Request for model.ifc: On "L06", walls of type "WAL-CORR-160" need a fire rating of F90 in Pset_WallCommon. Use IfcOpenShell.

First a look at what the model holds.

```python
import ifcopenshell
import ifcopenshell.util.element

model = ifcopenshell.open("model.ifc")
print(model.schema)
storey = next(s for s in model.by_type("IfcBuildingStorey") if s.Name == "L06")
walls = [e for e in ifcopenshell.util.element.get_decomposition(storey) if e.is_a("IfcWall")]
seen = {}
for e in walls:
    element_type = ifcopenshell.util.element.get_type(e)
    key = (element_type.Name if element_type != e and element_type else None, ifcopenshell.util.element.get_pset(e, "Pset_WallCommon", "FireRating"))
    seen[key] = seen.get(key, 0) + 1
for (name, value), count in sorted(seen.items(), key=str):
    print(count, "x", name, "|", value)
```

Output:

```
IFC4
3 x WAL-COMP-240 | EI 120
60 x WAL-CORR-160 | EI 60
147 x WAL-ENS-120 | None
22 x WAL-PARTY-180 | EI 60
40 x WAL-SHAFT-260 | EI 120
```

```python
import ifcopenshell
import ifcopenshell.api.pset
import ifcopenshell.util.element

model = ifcopenshell.open("model.ifc")

storey = next(s for s in model.by_type("IfcBuildingStorey") if s.Name == "L06")
walls = [e for e in ifcopenshell.util.element.get_decomposition(storey) if e.is_a("IfcWall")]

count = 0
for e in walls:
    element_type = ifcopenshell.util.element.get_type(e)
    if element_type in (None, e) or element_type.Name != "WAL-CORR-160":
        continue
    # add_pset returns the element's existing set when there is one.
    pset = ifcopenshell.api.pset.add_pset(model, product=e, name="Pset_WallCommon")
    ifcopenshell.api.pset.edit_pset(model, pset=pset, properties={"FireRating": "F90"})
    count += 1

print(count, "walls updated")

model.write("model_updated.ifc")
```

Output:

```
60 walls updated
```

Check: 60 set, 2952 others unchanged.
